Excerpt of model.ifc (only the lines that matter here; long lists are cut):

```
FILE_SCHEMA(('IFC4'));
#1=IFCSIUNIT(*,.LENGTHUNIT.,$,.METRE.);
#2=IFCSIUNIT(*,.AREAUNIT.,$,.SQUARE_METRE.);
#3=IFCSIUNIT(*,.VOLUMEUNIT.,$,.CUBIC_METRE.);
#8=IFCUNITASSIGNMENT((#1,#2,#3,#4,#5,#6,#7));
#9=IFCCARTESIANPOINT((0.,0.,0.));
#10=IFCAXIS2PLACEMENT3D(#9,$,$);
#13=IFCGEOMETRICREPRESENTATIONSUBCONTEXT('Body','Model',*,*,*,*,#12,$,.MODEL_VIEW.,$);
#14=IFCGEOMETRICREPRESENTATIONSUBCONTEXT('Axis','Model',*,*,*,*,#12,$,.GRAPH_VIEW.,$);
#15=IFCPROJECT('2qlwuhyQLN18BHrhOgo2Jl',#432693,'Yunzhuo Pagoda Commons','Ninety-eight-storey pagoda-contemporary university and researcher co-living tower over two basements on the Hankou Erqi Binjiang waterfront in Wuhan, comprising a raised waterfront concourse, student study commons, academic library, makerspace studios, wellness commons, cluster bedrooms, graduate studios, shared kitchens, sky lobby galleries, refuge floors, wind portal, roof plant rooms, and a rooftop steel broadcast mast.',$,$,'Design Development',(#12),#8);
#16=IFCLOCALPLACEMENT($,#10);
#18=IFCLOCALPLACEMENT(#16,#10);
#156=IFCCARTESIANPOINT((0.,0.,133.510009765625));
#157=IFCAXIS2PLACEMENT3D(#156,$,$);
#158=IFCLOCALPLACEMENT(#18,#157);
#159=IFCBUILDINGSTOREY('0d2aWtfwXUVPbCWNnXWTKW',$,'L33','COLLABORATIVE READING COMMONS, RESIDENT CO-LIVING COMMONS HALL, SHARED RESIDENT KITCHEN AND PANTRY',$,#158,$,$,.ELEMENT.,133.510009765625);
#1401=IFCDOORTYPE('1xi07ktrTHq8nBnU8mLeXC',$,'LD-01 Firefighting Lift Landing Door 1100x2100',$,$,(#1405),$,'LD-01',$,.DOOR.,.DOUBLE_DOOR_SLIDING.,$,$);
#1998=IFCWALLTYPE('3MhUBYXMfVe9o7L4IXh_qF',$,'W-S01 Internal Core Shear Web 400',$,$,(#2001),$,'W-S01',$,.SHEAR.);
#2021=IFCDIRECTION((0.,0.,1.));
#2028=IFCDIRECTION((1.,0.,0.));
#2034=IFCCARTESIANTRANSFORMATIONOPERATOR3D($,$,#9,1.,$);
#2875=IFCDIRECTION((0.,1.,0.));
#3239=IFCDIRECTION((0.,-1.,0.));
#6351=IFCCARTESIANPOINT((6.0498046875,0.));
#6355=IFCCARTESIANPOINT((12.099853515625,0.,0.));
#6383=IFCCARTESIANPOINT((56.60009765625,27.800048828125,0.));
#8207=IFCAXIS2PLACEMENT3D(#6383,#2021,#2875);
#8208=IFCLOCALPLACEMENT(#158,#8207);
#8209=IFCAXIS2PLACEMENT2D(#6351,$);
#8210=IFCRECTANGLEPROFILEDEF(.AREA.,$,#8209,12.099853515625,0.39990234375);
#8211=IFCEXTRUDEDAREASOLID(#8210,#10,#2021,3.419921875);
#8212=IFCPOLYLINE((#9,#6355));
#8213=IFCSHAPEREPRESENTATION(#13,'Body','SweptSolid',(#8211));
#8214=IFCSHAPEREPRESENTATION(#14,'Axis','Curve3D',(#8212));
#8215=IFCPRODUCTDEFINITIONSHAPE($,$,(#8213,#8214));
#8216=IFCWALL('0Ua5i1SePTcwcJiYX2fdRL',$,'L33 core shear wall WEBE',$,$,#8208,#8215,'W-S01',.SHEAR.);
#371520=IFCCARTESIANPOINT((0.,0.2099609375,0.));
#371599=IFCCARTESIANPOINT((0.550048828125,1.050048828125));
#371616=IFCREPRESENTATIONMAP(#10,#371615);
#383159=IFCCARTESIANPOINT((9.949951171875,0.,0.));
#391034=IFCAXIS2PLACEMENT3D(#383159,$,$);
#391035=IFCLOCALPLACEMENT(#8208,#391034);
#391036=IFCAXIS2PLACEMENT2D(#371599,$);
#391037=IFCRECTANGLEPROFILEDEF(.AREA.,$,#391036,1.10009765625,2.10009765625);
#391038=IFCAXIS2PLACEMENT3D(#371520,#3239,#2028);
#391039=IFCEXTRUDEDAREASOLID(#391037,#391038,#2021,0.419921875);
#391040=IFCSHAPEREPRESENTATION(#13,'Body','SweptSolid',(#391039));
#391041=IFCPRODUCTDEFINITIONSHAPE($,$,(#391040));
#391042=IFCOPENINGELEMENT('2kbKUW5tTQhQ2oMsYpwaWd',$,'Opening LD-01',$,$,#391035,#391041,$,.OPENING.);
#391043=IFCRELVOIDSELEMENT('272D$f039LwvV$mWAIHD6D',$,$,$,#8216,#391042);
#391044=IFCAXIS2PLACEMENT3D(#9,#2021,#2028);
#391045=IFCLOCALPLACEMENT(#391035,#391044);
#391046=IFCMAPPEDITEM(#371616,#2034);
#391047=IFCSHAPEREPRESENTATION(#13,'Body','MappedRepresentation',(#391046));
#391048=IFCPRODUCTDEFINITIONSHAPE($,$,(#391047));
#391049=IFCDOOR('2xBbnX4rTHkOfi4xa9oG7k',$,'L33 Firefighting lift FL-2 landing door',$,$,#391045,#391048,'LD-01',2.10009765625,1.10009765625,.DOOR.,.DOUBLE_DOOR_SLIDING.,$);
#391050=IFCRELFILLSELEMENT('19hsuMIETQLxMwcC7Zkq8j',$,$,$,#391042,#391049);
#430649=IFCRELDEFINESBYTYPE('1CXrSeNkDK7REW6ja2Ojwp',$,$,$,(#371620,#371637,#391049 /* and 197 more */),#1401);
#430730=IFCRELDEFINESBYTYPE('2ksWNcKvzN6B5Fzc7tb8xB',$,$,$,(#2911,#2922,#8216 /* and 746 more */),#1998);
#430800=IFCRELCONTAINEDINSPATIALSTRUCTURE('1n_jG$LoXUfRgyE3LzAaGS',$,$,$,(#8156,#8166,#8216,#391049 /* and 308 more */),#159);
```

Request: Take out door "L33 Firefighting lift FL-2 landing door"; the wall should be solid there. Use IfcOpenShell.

```python
import ifcopenshell
import ifcopenshell.api.feature
import ifcopenshell.api.root
import ifcopenshell.geom
import ifcopenshell.util.shape

model = ifcopenshell.open("model.ifc")
settings = ifcopenshell.geom.settings()


def volume(element):
    """Net volume in cubic metres, openings subtracted."""
    shape = ifcopenshell.geom.create_shape(settings, element)
    return ifcopenshell.util.shape.get_volume(shape.geometry)


door = model.by_guid("2xBbnX4rTHkOfi4xa9oG7k")
opening = door.FillsVoids[0].RelatingOpeningElement
wall = opening.VoidsElements[0].RelatingBuildingElement
before = volume(wall)

ifcopenshell.api.root.remove_product(model, product=door)
ifcopenshell.api.feature.remove_feature(model, feature=opening)

after = volume(wall)

print(f"wall volume {before:.3f} -> {after:.3f} m3")

model.write("model_rev.ifc")
```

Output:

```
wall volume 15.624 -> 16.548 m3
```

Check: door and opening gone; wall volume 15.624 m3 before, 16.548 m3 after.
